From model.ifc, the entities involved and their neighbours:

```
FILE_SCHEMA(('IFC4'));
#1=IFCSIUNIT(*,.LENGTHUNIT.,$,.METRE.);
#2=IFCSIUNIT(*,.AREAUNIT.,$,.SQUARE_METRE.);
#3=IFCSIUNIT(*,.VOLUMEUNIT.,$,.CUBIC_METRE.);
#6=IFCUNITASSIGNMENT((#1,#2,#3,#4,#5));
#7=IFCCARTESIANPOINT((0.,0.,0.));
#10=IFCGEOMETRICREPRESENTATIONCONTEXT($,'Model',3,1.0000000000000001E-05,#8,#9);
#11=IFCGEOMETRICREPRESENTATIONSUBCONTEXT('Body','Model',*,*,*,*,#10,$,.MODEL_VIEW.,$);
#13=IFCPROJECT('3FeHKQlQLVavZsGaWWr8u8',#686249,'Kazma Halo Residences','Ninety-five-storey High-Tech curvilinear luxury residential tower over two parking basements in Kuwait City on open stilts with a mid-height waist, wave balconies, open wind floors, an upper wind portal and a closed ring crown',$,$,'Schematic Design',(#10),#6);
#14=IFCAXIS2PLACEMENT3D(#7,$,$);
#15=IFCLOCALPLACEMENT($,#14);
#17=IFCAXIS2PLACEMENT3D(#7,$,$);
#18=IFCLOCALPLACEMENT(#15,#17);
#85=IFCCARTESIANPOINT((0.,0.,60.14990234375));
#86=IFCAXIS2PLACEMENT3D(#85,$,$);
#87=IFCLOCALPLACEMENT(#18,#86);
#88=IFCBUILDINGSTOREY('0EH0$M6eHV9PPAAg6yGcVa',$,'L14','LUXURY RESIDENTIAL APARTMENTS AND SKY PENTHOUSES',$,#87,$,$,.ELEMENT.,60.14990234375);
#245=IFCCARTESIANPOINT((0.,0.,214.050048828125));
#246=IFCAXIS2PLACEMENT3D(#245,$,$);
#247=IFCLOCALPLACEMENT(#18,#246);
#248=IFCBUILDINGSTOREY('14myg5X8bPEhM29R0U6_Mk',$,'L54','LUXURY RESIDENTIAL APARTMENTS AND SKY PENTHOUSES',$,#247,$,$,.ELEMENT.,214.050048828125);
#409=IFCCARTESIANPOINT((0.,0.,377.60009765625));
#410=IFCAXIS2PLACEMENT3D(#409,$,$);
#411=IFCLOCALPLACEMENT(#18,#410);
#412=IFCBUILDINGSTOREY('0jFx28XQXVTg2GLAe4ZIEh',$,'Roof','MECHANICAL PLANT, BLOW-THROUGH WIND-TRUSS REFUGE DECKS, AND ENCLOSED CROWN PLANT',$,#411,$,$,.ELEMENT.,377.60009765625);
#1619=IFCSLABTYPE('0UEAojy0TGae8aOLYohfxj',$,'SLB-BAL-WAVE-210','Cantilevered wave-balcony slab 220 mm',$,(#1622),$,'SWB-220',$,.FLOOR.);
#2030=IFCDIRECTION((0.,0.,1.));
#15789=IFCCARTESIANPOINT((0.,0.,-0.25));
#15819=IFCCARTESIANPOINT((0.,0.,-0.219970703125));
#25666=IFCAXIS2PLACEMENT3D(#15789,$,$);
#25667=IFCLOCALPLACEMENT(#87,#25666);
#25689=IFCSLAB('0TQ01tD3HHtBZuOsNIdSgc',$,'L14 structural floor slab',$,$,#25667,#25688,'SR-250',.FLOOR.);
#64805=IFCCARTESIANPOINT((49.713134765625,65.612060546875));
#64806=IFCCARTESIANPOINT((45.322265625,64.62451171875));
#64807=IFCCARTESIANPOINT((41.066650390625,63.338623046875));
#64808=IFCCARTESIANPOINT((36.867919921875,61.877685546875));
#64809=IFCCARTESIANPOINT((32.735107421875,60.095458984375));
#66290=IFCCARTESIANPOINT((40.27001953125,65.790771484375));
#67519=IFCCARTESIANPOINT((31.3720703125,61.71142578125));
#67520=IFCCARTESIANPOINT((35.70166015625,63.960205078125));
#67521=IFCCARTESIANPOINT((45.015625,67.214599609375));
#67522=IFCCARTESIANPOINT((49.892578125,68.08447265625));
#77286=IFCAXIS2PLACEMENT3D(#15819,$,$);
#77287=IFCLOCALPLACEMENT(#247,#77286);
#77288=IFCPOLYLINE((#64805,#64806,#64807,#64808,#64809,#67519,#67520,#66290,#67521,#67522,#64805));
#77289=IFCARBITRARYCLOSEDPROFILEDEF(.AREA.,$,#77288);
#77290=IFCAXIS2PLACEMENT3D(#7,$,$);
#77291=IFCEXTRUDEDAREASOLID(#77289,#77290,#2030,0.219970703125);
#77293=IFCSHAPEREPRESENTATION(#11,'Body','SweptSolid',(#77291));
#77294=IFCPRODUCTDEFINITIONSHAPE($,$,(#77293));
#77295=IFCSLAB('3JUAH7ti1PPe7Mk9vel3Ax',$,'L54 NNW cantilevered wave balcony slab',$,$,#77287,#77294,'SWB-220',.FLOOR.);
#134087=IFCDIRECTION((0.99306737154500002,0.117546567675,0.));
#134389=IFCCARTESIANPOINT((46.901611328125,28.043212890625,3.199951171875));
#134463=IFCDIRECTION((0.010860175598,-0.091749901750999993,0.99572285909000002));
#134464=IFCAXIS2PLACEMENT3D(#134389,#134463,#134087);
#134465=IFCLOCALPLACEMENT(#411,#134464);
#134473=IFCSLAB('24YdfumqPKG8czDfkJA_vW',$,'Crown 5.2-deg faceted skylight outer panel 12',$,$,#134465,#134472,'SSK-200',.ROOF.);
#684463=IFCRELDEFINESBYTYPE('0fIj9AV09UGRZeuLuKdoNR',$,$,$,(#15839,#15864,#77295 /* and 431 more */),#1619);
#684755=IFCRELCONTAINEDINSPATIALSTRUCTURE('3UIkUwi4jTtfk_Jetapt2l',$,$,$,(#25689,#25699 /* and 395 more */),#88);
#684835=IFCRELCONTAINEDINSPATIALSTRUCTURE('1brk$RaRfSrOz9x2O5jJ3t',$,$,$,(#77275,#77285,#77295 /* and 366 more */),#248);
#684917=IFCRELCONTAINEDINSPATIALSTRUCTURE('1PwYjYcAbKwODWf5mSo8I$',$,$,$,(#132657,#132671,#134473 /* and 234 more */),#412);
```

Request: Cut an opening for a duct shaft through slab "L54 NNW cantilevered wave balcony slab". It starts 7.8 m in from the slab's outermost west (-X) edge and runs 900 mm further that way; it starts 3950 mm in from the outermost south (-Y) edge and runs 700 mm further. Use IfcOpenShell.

```python
import numpy as np
import ifcopenshell
import ifcopenshell.api.feature
import ifcopenshell.api.geometry
import ifcopenshell.api.root
import ifcopenshell.geom
import ifcopenshell.util.placement
import ifcopenshell.util.representation
import ifcopenshell.util.shape
import ifcopenshell.util.unit

model = ifcopenshell.open("model.ifc")
unit_scale = ifcopenshell.util.unit.calculate_unit_scale(model)
settings = ifcopenshell.geom.settings()


def volume(element):
    """Net volume in cubic metres, openings subtracted."""
    shape = ifcopenshell.geom.create_shape(settings, element)
    return ifcopenshell.util.shape.get_volume(shape.geometry)


slab = model.by_id(77295)
before = volume(slab)

# Extent in the slab's own axes, in metres. The edges named are its -X and -Y sides.
slab_shape = ifcopenshell.geom.create_shape(settings, slab)
vertices = ifcopenshell.util.shape.get_vertices(slab_shape.geometry)
x_min, y_min, bottom = vertices.min(axis=0)
top = vertices[:, 2].max()

opening = ifcopenshell.api.root.create_entity(model, ifc_class="IfcOpeningElement", name="Duct shaft opening", predefined_type="OPENING")
context = ifcopenshell.util.representation.get_context(model, "Model", "Body", "MODEL_VIEW")
width, depth = 0.9, 0.7
outline = [(0.0, 0.0), (width, 0.0), (width, depth), (0.0, depth), (0.0, 0.0)]
# Overshoot both faces by 50 mm so the cut is clean.
shape = ifcopenshell.api.geometry.add_slab_representation(
    model, context=context, depth=top - bottom + 0.1, polyline=outline
)
ifcopenshell.api.geometry.assign_representation(model, product=opening, representation=shape)

matrix = ifcopenshell.util.placement.get_local_placement(slab.ObjectPlacement)
matrix[:, 3] = matrix @ np.append(np.array([x_min + 7.8, y_min + 3.95, bottom - 0.05]) / unit_scale, 1.0)
ifcopenshell.api.geometry.edit_object_placement(model, product=opening, matrix=matrix, is_si=False)
ifcopenshell.api.feature.add_feature(model, feature=opening, element=slab)

after = volume(slab)

print(f"slab volume {before:.3f} -> {after:.3f} m3")

model.write("model_rev.ifc")
```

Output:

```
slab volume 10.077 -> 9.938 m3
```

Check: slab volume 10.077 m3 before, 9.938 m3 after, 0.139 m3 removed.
